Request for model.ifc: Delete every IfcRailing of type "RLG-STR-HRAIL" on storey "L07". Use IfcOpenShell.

First a look at what the model holds.

```python
import ifcopenshell
import ifcopenshell.util.element

model = ifcopenshell.open("model.ifc")
print(model.schema)
storey = next(s for s in model.by_type("IfcBuildingStorey") if s.Name == "L07")
railings = [e for e in ifcopenshell.util.element.get_decomposition(storey) if e.is_a("IfcRailing")]
seen = {}
for e in railings:
    element_type = ifcopenshell.util.element.get_type(e)
    name = element_type.Name if element_type not in (None, e) else None
    seen[name] = seen.get(name, 0) + 1
for name, count in sorted(seen.items(), key=str):
    print(count, "x", name)
```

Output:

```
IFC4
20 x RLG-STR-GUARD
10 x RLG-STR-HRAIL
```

```python
import ifcopenshell
import ifcopenshell.api.root
import ifcopenshell.util.element

model = ifcopenshell.open("model.ifc")

storey = next(s for s in model.by_type("IfcBuildingStorey") if s.Name == "L07")
railings = [e for e in ifcopenshell.util.element.get_decomposition(storey) if e.is_a("IfcRailing")]
targets = [e for e in railings if (t := ifcopenshell.util.element.get_type(e)) not in (None, e) and t.Name == "RLG-STR-HRAIL"]

for e in targets:
    ifcopenshell.api.root.remove_product(model, product=e)
print(len(targets), "removed")

model.write("model_updated.ifc")
```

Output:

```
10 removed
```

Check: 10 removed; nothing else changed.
